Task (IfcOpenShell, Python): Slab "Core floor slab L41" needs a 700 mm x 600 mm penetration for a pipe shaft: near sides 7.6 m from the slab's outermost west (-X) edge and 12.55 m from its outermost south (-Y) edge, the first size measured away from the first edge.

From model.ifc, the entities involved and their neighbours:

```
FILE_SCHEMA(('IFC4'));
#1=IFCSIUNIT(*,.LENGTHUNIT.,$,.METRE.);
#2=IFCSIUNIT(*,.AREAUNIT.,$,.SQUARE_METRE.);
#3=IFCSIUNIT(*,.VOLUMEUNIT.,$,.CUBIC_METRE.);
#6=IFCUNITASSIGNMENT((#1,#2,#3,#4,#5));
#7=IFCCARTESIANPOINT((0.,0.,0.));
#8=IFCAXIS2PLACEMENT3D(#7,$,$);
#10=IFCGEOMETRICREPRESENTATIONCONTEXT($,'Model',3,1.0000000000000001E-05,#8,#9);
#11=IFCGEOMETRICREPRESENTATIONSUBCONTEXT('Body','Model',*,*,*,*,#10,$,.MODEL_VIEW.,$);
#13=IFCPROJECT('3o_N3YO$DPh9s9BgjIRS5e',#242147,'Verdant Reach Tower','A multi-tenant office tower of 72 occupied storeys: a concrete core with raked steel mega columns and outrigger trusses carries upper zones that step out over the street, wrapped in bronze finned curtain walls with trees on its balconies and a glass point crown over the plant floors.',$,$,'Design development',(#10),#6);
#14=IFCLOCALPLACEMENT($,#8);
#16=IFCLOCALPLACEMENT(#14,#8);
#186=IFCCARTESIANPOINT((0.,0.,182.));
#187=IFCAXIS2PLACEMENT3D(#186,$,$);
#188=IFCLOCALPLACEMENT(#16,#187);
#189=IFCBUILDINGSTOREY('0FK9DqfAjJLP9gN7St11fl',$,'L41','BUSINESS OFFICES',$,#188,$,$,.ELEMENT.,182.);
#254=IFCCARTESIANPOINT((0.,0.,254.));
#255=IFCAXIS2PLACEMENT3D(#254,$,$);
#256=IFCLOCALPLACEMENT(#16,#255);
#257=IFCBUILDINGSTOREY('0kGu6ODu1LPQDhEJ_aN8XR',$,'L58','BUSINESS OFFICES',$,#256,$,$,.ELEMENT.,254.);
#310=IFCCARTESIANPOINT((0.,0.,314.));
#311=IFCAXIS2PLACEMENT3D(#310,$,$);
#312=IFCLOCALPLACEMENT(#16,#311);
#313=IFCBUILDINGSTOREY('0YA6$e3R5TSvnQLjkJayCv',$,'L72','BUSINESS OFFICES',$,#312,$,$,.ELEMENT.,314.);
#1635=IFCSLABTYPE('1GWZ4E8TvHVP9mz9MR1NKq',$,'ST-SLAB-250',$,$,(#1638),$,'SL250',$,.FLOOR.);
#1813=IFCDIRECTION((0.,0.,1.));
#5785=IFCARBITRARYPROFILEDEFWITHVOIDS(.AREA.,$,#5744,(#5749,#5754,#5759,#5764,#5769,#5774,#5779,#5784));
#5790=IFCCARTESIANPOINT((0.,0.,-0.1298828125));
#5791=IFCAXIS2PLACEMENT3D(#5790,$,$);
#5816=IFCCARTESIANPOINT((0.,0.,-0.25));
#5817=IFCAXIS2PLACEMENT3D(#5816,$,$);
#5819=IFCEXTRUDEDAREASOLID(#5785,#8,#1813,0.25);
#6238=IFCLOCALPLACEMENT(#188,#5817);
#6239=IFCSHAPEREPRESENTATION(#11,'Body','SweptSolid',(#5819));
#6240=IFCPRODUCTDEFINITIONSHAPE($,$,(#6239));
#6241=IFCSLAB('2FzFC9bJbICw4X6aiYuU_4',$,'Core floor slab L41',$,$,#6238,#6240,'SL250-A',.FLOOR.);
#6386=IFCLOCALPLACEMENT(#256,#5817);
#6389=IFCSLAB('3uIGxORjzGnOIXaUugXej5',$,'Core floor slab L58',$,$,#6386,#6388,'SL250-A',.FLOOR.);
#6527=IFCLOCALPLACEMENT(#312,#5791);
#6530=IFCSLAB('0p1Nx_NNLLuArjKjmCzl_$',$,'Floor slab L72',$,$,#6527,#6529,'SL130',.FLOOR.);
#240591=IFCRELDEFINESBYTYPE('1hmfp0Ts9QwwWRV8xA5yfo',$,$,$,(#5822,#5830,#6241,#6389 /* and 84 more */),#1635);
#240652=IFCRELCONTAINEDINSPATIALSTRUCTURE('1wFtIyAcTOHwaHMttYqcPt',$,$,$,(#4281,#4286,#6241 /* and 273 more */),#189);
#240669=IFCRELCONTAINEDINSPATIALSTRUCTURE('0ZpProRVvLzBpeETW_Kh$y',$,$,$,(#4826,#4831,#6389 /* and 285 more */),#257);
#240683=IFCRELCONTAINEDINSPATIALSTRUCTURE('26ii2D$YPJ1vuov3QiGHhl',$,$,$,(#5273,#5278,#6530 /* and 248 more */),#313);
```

```python
import numpy as np
import ifcopenshell
import ifcopenshell.api.feature
import ifcopenshell.api.geometry
import ifcopenshell.api.root
import ifcopenshell.geom
import ifcopenshell.util.placement
import ifcopenshell.util.representation
import ifcopenshell.util.shape
import ifcopenshell.util.unit

model = ifcopenshell.open("model.ifc")
unit_scale = ifcopenshell.util.unit.calculate_unit_scale(model)
settings = ifcopenshell.geom.settings()


def volume(element):
    """Net volume in cubic metres, openings subtracted."""
    shape = ifcopenshell.geom.create_shape(settings, element)
    return ifcopenshell.util.shape.get_volume(shape.geometry)


slab = model.by_guid("2FzFC9bJbICw4X6aiYuU_4")
before = volume(slab)

# Extent in the slab's own axes, in metres. The edges named are its -X and -Y sides.
slab_shape = ifcopenshell.geom.create_shape(settings, slab)
vertices = ifcopenshell.util.shape.get_vertices(slab_shape.geometry)
x_min, y_min, bottom = vertices.min(axis=0)
top = vertices[:, 2].max()

opening = ifcopenshell.api.root.create_entity(model, ifc_class="IfcOpeningElement", name="Pipe shaft opening", predefined_type="OPENING")
context = ifcopenshell.util.representation.get_context(model, "Model", "Body", "MODEL_VIEW")
width, depth = 0.7, 0.6
outline = [(0.0, 0.0), (width, 0.0), (width, depth), (0.0, depth), (0.0, 0.0)]
# Overshoot both faces by 50 mm so the cut is clean.
shape = ifcopenshell.api.geometry.add_slab_representation(
    model, context=context, depth=top - bottom + 0.1, polyline=outline
)
ifcopenshell.api.geometry.assign_representation(model, product=opening, representation=shape)

matrix = ifcopenshell.util.placement.get_local_placement(slab.ObjectPlacement)
matrix[:, 3] = matrix @ np.append(np.array([x_min + 7.6, y_min + 12.55, bottom - 0.05]) / unit_scale, 1.0)
ifcopenshell.api.geometry.edit_object_placement(model, product=opening, matrix=matrix, is_si=False)
ifcopenshell.api.feature.add_feature(model, feature=opening, element=slab)

after = volume(slab)

print(f"slab volume {before:.3f} -> {after:.3f} m3")

model.write("model_edited.ifc")
```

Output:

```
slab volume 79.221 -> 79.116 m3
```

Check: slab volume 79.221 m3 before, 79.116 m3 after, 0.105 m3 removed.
